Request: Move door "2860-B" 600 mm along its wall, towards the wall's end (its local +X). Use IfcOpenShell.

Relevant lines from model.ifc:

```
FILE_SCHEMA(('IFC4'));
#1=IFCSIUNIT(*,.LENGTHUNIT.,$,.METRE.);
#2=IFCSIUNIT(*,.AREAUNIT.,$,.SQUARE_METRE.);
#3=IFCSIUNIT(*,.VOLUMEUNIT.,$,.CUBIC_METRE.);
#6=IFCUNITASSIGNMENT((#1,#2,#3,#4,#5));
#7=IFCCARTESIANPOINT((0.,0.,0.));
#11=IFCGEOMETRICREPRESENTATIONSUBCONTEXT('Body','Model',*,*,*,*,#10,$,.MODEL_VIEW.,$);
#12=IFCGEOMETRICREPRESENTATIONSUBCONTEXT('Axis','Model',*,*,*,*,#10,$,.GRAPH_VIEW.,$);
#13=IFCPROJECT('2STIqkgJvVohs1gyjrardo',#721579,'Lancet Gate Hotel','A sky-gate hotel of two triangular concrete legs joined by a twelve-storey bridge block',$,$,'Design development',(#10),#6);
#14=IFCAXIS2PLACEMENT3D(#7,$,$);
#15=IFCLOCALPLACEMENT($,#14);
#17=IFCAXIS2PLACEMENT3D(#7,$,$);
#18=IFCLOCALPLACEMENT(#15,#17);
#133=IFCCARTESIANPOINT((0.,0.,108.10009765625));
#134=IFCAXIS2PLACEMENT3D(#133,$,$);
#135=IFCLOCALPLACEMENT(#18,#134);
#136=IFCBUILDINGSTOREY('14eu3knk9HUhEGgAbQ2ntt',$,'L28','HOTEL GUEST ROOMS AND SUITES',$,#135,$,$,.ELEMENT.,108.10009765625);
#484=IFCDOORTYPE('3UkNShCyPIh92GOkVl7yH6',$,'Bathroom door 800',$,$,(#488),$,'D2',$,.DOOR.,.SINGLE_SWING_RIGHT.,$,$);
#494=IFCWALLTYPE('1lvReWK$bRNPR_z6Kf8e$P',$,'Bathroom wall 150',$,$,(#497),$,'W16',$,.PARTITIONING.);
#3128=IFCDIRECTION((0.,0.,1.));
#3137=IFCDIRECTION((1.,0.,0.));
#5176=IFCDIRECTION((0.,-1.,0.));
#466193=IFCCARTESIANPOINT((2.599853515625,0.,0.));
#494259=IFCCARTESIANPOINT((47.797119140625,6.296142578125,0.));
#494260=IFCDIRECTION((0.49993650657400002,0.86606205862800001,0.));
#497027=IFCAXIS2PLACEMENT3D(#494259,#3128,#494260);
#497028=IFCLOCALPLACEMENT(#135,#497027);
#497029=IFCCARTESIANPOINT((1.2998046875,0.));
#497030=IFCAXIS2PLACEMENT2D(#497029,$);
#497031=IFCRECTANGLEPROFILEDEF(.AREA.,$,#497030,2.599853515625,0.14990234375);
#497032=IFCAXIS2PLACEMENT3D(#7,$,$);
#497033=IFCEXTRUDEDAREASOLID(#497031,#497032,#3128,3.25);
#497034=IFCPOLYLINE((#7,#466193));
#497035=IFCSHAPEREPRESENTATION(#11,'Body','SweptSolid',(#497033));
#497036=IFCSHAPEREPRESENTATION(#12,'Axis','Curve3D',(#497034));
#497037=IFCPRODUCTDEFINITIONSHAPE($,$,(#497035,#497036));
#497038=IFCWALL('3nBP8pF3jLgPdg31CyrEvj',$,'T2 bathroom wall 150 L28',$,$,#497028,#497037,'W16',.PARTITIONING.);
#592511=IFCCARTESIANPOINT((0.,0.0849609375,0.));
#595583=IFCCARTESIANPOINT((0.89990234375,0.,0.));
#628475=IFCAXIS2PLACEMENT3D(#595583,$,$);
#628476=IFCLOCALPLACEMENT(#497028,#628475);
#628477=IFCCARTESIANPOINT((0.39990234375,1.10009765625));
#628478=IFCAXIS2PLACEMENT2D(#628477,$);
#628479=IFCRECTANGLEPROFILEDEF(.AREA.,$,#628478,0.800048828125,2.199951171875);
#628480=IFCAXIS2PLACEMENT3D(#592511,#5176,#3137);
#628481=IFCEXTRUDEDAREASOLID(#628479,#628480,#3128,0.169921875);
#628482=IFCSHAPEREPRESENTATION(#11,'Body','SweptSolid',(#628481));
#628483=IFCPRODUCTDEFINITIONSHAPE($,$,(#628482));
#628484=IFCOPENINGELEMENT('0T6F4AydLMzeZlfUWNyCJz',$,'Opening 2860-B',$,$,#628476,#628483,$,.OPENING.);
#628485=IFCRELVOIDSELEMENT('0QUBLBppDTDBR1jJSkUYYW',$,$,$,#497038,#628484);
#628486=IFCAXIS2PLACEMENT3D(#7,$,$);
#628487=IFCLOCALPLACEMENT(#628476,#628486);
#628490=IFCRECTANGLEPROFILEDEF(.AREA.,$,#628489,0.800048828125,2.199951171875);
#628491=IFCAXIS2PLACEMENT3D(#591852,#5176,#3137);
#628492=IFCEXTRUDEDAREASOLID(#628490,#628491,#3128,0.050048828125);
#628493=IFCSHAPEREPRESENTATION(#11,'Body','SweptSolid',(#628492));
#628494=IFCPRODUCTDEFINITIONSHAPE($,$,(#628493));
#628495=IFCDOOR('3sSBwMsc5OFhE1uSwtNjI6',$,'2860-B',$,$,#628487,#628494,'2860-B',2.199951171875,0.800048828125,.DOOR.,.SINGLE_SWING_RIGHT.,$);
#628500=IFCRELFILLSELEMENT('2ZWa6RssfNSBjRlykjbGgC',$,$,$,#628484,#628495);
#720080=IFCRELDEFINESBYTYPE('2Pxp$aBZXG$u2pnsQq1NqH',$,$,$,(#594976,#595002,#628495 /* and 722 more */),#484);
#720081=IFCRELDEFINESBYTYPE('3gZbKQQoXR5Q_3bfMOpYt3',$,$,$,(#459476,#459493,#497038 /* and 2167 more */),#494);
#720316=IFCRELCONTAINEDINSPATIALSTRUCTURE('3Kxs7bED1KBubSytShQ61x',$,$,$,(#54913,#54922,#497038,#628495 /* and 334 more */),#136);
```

```python
import ifcopenshell
import ifcopenshell.api.geometry
import ifcopenshell.util.placement
import ifcopenshell.util.unit

model = ifcopenshell.open("model.ifc")
unit_scale = ifcopenshell.util.unit.calculate_unit_scale(model)

door = model.by_guid("3sSBwMsc5OFhE1uSwtNjI6")
opening = door.FillsVoids[0].RelatingOpeningElement
wall = opening.VoidsElements[0].RelatingBuildingElement

wall_matrix = ifcopenshell.util.placement.get_local_placement(wall.ObjectPlacement)
shift = wall_matrix[:3, 0] * 0.6 / unit_scale
before = ifcopenshell.util.placement.get_local_placement(door.ObjectPlacement)[:3, 3].copy()

# The door is placed relative to its opening, so it follows when the opening moves.
matrix = ifcopenshell.util.placement.get_local_placement(opening.ObjectPlacement)
matrix[:3, 3] += shift
ifcopenshell.api.geometry.edit_object_placement(
    model, product=opening, matrix=matrix, is_si=False, should_transform_children=True
)

after = ifcopenshell.util.placement.get_local_placement(door.ObjectPlacement)[:3, 3]
print("door moved by", (after - before).round(3) + 0.0)

model.write("model_rev.ifc")
```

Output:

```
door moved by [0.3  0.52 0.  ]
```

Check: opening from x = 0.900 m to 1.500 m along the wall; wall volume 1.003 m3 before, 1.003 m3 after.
